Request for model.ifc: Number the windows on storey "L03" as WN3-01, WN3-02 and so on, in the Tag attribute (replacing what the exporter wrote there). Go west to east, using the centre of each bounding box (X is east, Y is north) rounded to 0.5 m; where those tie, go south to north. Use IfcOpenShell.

First a look at what the model holds.

```python
import ifcopenshell
import ifcopenshell.util.element
import ifcopenshell.util.placement

model = ifcopenshell.open("model.ifc")
print(model.schema)
storey = next(s for s in model.by_type("IfcBuildingStorey") if s.Name == "L03")
windows = [e for e in ifcopenshell.util.element.get_decomposition(storey) if e.is_a("IfcWindow")]
for e in sorted(windows, key=lambda e: e.id()):
    origin = ifcopenshell.util.placement.get_local_placement(e.ObjectPlacement)[:3, 3]
    print(e.id(), e.Tag, e.Name, origin.round(2) + 0.0, sep=" | ")
```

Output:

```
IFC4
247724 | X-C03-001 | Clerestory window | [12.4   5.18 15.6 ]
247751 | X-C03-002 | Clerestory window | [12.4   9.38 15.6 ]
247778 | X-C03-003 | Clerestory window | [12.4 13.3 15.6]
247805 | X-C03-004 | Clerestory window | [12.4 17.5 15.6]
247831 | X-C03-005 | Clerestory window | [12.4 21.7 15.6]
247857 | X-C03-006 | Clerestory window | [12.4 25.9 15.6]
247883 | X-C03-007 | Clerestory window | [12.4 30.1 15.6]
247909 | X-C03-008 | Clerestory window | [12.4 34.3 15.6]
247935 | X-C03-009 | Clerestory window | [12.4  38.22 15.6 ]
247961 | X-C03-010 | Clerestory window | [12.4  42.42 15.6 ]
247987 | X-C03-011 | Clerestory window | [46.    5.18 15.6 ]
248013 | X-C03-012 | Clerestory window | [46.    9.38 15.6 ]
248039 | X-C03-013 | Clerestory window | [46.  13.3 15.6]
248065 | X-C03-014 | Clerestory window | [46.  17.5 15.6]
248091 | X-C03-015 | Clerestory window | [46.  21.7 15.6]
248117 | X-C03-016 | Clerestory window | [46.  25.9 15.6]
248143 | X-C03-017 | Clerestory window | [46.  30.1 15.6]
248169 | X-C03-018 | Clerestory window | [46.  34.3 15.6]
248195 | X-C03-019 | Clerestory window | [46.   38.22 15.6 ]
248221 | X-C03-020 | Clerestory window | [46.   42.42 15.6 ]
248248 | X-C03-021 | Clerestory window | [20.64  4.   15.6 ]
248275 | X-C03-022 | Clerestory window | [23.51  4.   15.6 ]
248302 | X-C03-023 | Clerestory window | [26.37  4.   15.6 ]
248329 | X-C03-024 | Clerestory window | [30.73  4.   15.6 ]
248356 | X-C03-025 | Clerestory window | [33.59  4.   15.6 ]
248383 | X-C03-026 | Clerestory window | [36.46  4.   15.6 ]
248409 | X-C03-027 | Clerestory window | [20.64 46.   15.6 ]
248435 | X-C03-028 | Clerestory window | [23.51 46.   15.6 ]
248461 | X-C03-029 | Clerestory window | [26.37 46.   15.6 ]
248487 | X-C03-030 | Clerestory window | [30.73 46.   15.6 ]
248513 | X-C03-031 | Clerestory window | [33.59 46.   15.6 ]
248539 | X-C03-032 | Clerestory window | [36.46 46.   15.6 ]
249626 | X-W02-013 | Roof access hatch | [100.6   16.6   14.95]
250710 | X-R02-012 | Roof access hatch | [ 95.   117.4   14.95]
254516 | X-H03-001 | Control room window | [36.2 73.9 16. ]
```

```python
import ifcopenshell
import ifcopenshell.geom
import ifcopenshell.util.element
import ifcopenshell.util.shape

model = ifcopenshell.open("model.ifc")
settings = ifcopenshell.geom.settings()
settings.set("use-world-coords", True)


def centre(element):
    shape = ifcopenshell.geom.create_shape(settings, element)
    return ifcopenshell.util.shape.get_bbox_centroid(shape.geometry)


storey = next(s for s in model.by_type("IfcBuildingStorey") if s.Name == "L03")
windows = [e for e in ifcopenshell.util.element.get_decomposition(storey) if e.is_a("IfcWindow")]

# Insertion points can sit at a corner or the storey origin, so sort by the geometry (in metres).
centres = {e: centre(e) for e in windows}
windows.sort(key=lambda e: (round(centres[e][0] / 0.5), centres[e][1]))

for i, e in enumerate(windows, start=1):
    number = f"WN3-{i:02d}"
    e.Tag = number
    print(e.id(), number)

model.write("model_rev.ifc")
```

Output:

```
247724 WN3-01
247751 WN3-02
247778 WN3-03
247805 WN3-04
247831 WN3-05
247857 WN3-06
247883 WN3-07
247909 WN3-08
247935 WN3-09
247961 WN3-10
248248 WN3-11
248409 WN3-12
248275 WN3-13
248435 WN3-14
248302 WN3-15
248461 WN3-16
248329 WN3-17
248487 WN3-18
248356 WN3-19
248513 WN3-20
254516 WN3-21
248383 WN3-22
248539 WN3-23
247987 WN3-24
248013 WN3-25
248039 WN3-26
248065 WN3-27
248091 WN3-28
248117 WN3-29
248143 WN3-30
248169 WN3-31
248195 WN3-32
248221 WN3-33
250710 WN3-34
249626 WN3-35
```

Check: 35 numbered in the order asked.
